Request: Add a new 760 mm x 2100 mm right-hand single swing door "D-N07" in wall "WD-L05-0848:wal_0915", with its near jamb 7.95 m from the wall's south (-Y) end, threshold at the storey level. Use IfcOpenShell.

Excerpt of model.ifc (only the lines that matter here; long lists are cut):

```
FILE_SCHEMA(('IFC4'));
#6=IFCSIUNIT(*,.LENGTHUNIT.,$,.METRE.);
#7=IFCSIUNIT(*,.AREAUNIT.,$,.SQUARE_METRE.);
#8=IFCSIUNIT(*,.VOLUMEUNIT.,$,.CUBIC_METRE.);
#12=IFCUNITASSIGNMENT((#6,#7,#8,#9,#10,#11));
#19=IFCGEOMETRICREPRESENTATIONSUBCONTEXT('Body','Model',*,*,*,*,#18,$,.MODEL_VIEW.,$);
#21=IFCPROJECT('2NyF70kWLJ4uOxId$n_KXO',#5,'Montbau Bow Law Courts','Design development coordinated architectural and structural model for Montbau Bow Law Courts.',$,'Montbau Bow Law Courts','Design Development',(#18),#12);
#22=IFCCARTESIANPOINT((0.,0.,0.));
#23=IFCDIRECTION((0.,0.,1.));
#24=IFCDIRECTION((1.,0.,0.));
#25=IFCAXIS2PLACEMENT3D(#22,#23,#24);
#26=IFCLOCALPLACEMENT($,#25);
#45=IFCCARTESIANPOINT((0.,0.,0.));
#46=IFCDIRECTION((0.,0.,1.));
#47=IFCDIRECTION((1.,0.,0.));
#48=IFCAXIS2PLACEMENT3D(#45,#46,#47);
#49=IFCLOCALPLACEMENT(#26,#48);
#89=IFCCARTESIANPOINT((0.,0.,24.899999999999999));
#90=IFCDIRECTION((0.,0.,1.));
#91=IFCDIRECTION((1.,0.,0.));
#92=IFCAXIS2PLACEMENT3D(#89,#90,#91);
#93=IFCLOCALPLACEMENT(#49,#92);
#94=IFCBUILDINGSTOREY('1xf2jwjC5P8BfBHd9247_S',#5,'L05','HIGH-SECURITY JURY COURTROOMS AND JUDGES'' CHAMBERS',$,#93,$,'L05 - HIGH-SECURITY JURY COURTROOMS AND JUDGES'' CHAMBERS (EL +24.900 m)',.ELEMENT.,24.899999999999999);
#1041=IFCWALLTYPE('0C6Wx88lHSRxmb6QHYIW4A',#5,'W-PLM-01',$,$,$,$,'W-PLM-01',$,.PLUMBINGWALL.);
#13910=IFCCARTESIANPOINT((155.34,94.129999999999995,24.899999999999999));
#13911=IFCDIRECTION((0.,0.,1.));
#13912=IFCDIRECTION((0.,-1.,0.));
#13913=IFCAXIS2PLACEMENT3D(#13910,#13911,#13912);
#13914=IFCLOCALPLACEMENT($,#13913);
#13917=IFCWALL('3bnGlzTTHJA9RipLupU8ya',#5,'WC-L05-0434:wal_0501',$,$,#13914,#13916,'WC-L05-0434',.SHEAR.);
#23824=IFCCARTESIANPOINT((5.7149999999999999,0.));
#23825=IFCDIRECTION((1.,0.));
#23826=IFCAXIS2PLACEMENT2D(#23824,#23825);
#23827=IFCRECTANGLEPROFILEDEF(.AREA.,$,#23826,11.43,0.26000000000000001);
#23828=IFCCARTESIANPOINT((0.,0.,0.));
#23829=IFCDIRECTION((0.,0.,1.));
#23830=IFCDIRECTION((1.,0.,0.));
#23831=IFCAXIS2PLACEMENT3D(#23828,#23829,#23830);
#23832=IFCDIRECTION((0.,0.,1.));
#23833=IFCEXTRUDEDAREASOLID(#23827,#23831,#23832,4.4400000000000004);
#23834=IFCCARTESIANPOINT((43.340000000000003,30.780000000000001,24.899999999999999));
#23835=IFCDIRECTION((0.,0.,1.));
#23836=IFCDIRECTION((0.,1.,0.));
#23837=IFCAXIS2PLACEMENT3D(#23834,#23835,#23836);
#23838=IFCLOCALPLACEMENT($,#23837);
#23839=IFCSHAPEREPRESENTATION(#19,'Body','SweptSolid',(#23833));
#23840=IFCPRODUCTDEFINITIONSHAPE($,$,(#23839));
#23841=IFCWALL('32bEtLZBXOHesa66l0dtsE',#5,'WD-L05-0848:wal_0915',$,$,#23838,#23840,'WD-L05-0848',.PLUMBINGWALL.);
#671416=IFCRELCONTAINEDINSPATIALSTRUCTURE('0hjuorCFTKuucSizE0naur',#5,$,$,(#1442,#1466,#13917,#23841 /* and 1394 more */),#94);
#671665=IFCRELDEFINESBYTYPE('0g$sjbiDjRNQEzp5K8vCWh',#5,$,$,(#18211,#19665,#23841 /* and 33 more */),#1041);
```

```python
import numpy as np
import ifcopenshell
import ifcopenshell.api.feature
import ifcopenshell.api.geometry
import ifcopenshell.api.root
import ifcopenshell.api.spatial
import ifcopenshell.geom
import ifcopenshell.util.element
import ifcopenshell.util.placement
import ifcopenshell.util.representation
import ifcopenshell.util.shape
import ifcopenshell.util.unit

model = ifcopenshell.open("model.ifc")
unit_scale = ifcopenshell.util.unit.calculate_unit_scale(model)
settings = ifcopenshell.geom.settings()


def volume(element):
    """Net volume in cubic metres, openings subtracted."""
    shape = ifcopenshell.geom.create_shape(settings, element)
    return ifcopenshell.util.shape.get_volume(shape.geometry)


wall = model.by_id(23841)
storey = ifcopenshell.util.element.get_container(wall, ifc_class="IfcBuildingStorey")
context = ifcopenshell.util.representation.get_context(model, "Model", "Body", "MODEL_VIEW")
before = volume(wall)

width, height, from_end, sill = 0.76, 2.1, 7.95, 0.0  # metres

# The wall runs along its own X axis, and the end named is its -X end.
wall_shape = ifcopenshell.geom.create_shape(settings, wall)
x, y, z = ifcopenshell.util.shape.get_vertices(wall_shape.geometry).T
start = x.min() + from_end
face, thickness = float(y.min()), float(y.max() - y.min())
wall_matrix = ifcopenshell.util.placement.get_local_placement(wall.ObjectPlacement)
level = ifcopenshell.util.placement.get_local_placement(storey.ObjectPlacement)[2, 3]


def in_wall(x, y):
    """Placement at x, y metres in the wall's axes, at sill height."""
    matrix = wall_matrix.copy()
    matrix[:, 3] = wall_matrix @ np.array([x / unit_scale, y / unit_scale, 0.0, 1.0])
    matrix[2, 3] = level + sill / unit_scale
    return matrix


# Opening: a box that overshoots both wall faces by 50 mm.
opening = ifcopenshell.api.root.create_entity(model, ifc_class="IfcOpeningElement", predefined_type="OPENING")
box = ifcopenshell.api.geometry.add_wall_representation(
    model, context=context, length=width, height=height, thickness=thickness + 0.1
)
ifcopenshell.api.geometry.assign_representation(model, product=opening, representation=box)
ifcopenshell.api.geometry.edit_object_placement(model, product=opening, matrix=in_wall(start, face - 0.05), is_si=False)
ifcopenshell.api.feature.add_feature(model, feature=opening, element=wall)

door = ifcopenshell.api.root.create_entity(model, ifc_class="IfcDoor", name="D-N07", predefined_type="DOOR")
door.OverallWidth, door.OverallHeight = width / unit_scale, height / unit_scale
door.OperationType = "SINGLE_SWING_RIGHT"
body = ifcopenshell.api.geometry.add_door_representation(
    model,
    context=context,
    overall_width=door.OverallWidth,
    overall_height=door.OverallHeight,
    operation_type="SINGLE_SWING_RIGHT",
    lining_properties={"LiningDepth": thickness / unit_scale, "ThresholdDepth": thickness / unit_scale},
)
ifcopenshell.api.geometry.assign_representation(model, product=door, representation=body)
ifcopenshell.api.spatial.assign_container(model, products=[door], relating_structure=storey)
ifcopenshell.api.feature.add_filling(model, opening=opening, element=door)

# The lining spans the wall, so the door starts at the wall face.
ifcopenshell.api.geometry.edit_object_placement(model, product=door, matrix=in_wall(start, face), is_si=False)

after = volume(wall)

print(f"wall volume {before:.3f} -> {after:.3f} m3")

model.write("model_rev.ifc")
```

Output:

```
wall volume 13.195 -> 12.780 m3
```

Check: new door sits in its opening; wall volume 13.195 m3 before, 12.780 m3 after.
